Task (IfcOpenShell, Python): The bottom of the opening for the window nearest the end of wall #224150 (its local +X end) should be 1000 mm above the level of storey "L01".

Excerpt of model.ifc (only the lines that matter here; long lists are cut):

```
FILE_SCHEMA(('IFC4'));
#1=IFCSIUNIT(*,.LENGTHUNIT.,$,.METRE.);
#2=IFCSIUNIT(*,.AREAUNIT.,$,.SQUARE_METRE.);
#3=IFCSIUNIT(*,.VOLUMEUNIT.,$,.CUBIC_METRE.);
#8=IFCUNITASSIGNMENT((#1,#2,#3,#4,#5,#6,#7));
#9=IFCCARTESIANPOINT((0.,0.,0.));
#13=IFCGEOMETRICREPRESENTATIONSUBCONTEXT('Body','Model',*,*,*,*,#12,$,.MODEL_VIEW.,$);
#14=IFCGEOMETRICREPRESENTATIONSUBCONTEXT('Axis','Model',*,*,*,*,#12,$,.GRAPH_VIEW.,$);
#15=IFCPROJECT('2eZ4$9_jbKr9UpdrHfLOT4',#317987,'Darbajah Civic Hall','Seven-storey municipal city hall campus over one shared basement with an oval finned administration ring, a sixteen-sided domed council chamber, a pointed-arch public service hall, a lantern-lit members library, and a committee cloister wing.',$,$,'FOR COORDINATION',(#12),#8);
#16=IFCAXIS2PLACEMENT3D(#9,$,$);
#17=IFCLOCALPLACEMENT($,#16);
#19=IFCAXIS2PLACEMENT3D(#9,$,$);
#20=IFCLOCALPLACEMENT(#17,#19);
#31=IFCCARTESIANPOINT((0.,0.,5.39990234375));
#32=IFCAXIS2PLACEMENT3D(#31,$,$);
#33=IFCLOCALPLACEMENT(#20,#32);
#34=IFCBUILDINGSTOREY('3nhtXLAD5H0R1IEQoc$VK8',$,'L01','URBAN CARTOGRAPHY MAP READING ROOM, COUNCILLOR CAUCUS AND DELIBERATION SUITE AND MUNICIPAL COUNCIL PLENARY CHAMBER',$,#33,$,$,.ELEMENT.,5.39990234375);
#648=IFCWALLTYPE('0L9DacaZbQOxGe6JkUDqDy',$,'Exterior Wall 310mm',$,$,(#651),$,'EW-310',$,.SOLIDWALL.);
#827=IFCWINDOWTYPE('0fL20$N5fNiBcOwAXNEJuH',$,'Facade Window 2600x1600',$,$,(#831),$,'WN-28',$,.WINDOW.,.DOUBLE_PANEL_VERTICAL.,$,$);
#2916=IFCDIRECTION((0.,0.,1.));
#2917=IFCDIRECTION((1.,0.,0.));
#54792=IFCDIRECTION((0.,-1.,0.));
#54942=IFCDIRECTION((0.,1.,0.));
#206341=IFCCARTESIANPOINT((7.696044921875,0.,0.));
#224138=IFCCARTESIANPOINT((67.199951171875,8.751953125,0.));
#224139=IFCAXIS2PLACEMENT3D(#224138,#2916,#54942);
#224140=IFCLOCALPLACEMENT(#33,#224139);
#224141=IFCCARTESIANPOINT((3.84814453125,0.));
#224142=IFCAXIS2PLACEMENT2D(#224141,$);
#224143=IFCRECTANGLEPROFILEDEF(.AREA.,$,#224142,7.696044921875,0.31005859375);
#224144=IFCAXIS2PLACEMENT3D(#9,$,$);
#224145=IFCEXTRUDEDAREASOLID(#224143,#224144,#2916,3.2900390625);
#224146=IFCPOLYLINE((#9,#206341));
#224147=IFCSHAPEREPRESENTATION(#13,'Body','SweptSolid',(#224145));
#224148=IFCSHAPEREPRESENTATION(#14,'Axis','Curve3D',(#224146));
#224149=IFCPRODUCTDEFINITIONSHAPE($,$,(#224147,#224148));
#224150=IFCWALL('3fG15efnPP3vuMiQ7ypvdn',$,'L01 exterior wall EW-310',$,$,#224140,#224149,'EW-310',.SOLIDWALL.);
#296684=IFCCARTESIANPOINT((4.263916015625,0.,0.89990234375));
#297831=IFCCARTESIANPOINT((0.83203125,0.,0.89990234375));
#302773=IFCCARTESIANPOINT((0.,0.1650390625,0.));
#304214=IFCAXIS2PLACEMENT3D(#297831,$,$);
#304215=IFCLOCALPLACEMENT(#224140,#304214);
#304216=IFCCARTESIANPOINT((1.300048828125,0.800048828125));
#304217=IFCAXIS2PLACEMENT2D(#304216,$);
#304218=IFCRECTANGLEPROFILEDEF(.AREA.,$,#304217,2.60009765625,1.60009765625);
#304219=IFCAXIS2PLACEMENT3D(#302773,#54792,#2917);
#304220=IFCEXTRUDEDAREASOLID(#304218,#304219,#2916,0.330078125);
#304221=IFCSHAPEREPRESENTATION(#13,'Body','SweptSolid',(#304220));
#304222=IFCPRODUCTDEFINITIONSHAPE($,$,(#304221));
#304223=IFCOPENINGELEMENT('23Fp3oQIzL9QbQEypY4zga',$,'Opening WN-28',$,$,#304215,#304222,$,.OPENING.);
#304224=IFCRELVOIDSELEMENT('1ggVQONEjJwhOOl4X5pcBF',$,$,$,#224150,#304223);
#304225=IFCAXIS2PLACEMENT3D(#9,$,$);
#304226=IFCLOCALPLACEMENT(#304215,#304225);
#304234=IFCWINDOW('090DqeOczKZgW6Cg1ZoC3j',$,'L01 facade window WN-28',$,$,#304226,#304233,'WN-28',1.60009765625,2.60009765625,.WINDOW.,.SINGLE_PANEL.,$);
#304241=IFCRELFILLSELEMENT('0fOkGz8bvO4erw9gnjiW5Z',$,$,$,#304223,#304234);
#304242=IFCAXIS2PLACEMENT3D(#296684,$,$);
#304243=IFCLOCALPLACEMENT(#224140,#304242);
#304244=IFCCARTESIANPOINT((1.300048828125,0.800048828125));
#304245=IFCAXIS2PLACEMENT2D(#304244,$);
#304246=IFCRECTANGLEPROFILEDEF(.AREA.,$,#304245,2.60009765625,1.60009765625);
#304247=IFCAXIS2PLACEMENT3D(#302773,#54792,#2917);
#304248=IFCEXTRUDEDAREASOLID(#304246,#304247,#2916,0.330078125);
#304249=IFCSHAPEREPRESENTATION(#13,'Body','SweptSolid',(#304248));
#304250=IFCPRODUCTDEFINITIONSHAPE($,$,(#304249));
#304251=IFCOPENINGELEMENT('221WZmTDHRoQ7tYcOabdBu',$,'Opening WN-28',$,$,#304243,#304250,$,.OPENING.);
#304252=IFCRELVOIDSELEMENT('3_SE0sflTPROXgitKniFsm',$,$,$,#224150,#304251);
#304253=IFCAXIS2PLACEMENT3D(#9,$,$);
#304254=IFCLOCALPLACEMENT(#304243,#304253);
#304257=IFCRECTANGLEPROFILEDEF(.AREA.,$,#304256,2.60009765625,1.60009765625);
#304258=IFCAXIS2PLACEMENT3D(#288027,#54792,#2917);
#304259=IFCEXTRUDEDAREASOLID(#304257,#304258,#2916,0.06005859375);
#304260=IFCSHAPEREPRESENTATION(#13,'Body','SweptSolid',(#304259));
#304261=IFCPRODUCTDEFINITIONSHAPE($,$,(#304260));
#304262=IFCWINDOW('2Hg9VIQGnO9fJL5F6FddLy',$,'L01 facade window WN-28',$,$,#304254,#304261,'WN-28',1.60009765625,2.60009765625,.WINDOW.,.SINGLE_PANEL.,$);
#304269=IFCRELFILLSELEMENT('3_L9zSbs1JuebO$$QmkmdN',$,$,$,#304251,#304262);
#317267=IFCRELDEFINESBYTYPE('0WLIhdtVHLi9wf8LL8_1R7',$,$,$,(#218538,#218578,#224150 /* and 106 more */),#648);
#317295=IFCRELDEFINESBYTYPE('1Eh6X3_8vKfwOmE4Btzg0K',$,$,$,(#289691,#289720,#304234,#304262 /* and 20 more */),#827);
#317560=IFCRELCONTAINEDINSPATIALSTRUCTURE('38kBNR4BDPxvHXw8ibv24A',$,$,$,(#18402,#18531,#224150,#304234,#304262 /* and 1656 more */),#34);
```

```python
import numpy as np
import ifcopenshell
import ifcopenshell.api.geometry
import ifcopenshell.geom
import ifcopenshell.util.element
import ifcopenshell.util.placement
import ifcopenshell.util.shape
import ifcopenshell.util.unit

model = ifcopenshell.open("model.ifc")
unit_scale = ifcopenshell.util.unit.calculate_unit_scale(model)

window = model.by_guid("2Hg9VIQGnO9fJL5F6FddLy")
opening = window.FillsVoids[0].RelatingOpeningElement
storey = ifcopenshell.util.element.get_container(window, ifc_class="IfcBuildingStorey")
level = ifcopenshell.util.placement.get_local_placement(storey.ObjectPlacement)[2, 3]

# The opening's origin need not be at the sill, so measure its lowest point.
shape = ifcopenshell.geom.create_shape(ifcopenshell.geom.settings(), opening)
bottom = ifcopenshell.util.shape.get_shape_bottom_elevation(shape, shape.geometry) / unit_scale
dz = level + 1 / unit_scale - bottom

shift = np.array([0.0, 0.0, dz])
# The window is placed relative to its opening, so it follows when the opening moves.
matrix = ifcopenshell.util.placement.get_local_placement(opening.ObjectPlacement)
matrix[:3, 3] += shift
ifcopenshell.api.geometry.edit_object_placement(
    model, product=opening, matrix=matrix, is_si=False, should_transform_children=True
)

print(f"moved by {dz * unit_scale:+.3f} m")

model.write("model-out.ifc")
```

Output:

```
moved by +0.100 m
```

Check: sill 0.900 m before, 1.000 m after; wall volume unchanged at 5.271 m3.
